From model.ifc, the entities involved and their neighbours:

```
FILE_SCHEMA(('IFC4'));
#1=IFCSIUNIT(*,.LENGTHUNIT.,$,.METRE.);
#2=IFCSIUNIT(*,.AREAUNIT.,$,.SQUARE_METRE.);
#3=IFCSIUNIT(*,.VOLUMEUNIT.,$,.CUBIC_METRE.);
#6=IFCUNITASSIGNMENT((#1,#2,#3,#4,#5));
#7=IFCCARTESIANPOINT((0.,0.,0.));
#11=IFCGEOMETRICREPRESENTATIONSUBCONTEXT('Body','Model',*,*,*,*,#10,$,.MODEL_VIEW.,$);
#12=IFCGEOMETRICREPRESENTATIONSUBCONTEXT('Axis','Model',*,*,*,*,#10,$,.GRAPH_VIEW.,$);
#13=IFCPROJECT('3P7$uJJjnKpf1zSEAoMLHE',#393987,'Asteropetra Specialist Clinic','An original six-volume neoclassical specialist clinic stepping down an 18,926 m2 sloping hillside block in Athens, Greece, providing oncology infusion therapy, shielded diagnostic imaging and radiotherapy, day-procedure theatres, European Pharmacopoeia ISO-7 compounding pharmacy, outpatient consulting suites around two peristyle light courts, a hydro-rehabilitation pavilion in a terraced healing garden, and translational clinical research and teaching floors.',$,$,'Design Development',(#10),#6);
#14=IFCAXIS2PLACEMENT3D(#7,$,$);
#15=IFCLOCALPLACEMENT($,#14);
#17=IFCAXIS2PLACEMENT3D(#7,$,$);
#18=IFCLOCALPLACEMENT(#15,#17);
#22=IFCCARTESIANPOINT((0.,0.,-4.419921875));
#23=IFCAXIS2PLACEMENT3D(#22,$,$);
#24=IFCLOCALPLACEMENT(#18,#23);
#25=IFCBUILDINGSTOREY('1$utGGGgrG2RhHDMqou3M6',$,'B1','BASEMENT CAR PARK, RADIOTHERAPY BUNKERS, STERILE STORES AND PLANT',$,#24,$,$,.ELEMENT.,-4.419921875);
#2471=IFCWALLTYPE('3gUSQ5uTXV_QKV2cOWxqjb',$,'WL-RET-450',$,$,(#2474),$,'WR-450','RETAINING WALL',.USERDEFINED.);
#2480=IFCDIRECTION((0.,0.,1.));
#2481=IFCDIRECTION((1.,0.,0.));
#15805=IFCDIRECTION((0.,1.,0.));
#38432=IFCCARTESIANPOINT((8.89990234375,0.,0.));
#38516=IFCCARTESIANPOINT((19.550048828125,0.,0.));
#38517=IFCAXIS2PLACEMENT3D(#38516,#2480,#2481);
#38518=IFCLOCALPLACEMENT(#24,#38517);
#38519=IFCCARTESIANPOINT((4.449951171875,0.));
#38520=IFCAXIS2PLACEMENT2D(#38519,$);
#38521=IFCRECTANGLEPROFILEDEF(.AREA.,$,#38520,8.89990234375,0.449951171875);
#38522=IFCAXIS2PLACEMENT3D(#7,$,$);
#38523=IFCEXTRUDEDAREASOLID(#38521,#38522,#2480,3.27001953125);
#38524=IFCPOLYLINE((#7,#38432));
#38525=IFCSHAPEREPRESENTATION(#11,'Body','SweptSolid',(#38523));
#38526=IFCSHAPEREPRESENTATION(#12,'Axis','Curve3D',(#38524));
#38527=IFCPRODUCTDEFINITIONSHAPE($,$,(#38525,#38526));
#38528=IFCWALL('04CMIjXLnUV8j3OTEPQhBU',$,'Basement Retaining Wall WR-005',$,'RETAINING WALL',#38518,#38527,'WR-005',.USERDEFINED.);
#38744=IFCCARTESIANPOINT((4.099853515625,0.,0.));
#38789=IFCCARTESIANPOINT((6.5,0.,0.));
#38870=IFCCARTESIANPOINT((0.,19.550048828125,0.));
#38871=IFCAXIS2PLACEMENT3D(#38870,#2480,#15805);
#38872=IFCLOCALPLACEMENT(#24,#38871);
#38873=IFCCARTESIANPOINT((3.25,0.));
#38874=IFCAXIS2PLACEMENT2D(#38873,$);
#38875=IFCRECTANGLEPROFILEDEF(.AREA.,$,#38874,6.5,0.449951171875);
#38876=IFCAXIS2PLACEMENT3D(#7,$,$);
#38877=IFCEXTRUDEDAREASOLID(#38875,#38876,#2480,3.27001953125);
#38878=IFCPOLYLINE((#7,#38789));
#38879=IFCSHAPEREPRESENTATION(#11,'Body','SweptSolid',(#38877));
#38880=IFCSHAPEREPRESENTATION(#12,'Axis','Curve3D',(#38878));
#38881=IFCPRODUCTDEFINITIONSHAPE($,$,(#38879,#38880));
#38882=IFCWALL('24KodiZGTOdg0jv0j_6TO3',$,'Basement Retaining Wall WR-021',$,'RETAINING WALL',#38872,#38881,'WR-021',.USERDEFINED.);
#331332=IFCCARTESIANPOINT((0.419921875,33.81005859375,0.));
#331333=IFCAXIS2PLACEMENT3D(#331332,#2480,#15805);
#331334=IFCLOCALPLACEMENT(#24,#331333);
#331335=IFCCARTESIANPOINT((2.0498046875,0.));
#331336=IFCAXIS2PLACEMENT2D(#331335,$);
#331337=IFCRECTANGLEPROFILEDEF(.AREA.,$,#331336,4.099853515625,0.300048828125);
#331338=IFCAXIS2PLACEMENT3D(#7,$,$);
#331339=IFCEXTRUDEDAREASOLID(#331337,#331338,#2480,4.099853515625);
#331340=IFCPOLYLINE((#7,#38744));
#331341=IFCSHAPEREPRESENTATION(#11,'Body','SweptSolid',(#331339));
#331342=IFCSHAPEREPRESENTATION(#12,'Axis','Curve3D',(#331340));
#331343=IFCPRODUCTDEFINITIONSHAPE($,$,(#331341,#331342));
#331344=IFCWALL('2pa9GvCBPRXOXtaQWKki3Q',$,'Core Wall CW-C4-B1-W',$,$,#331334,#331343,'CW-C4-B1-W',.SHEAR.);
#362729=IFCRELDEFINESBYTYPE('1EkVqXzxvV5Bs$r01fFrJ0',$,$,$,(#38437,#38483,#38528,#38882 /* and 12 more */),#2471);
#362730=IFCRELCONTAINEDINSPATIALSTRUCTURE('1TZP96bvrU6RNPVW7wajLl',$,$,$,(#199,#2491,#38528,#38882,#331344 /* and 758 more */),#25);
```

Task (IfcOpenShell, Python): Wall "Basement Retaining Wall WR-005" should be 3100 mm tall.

```python
import ifcopenshell
import ifcopenshell.geom
import ifcopenshell.util.representation
import ifcopenshell.util.shape
import ifcopenshell.util.unit

model = ifcopenshell.open("model.ifc")
unit_scale = ifcopenshell.util.unit.calculate_unit_scale(model)
settings = ifcopenshell.geom.settings()


def volume(element):
    """Net volume in cubic metres, openings subtracted."""
    shape = ifcopenshell.geom.create_shape(settings, element)
    return ifcopenshell.util.shape.get_volume(shape.geometry)


wall = model.by_id(38528)
before = volume(wall)

body = ifcopenshell.util.representation.get_representation(wall, "Model", "Body")
solid = body.Items[0]
old_height = solid.Depth
solid.Depth = 3.1 / unit_scale
after = volume(wall)

print(f"height {old_height:g} -> {solid.Depth:g}, volume {before:.3f} -> {after:.3f} m3")

model.write("model-out.ifc")
```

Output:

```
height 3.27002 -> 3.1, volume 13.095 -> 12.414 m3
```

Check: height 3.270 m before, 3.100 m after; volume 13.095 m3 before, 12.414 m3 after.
